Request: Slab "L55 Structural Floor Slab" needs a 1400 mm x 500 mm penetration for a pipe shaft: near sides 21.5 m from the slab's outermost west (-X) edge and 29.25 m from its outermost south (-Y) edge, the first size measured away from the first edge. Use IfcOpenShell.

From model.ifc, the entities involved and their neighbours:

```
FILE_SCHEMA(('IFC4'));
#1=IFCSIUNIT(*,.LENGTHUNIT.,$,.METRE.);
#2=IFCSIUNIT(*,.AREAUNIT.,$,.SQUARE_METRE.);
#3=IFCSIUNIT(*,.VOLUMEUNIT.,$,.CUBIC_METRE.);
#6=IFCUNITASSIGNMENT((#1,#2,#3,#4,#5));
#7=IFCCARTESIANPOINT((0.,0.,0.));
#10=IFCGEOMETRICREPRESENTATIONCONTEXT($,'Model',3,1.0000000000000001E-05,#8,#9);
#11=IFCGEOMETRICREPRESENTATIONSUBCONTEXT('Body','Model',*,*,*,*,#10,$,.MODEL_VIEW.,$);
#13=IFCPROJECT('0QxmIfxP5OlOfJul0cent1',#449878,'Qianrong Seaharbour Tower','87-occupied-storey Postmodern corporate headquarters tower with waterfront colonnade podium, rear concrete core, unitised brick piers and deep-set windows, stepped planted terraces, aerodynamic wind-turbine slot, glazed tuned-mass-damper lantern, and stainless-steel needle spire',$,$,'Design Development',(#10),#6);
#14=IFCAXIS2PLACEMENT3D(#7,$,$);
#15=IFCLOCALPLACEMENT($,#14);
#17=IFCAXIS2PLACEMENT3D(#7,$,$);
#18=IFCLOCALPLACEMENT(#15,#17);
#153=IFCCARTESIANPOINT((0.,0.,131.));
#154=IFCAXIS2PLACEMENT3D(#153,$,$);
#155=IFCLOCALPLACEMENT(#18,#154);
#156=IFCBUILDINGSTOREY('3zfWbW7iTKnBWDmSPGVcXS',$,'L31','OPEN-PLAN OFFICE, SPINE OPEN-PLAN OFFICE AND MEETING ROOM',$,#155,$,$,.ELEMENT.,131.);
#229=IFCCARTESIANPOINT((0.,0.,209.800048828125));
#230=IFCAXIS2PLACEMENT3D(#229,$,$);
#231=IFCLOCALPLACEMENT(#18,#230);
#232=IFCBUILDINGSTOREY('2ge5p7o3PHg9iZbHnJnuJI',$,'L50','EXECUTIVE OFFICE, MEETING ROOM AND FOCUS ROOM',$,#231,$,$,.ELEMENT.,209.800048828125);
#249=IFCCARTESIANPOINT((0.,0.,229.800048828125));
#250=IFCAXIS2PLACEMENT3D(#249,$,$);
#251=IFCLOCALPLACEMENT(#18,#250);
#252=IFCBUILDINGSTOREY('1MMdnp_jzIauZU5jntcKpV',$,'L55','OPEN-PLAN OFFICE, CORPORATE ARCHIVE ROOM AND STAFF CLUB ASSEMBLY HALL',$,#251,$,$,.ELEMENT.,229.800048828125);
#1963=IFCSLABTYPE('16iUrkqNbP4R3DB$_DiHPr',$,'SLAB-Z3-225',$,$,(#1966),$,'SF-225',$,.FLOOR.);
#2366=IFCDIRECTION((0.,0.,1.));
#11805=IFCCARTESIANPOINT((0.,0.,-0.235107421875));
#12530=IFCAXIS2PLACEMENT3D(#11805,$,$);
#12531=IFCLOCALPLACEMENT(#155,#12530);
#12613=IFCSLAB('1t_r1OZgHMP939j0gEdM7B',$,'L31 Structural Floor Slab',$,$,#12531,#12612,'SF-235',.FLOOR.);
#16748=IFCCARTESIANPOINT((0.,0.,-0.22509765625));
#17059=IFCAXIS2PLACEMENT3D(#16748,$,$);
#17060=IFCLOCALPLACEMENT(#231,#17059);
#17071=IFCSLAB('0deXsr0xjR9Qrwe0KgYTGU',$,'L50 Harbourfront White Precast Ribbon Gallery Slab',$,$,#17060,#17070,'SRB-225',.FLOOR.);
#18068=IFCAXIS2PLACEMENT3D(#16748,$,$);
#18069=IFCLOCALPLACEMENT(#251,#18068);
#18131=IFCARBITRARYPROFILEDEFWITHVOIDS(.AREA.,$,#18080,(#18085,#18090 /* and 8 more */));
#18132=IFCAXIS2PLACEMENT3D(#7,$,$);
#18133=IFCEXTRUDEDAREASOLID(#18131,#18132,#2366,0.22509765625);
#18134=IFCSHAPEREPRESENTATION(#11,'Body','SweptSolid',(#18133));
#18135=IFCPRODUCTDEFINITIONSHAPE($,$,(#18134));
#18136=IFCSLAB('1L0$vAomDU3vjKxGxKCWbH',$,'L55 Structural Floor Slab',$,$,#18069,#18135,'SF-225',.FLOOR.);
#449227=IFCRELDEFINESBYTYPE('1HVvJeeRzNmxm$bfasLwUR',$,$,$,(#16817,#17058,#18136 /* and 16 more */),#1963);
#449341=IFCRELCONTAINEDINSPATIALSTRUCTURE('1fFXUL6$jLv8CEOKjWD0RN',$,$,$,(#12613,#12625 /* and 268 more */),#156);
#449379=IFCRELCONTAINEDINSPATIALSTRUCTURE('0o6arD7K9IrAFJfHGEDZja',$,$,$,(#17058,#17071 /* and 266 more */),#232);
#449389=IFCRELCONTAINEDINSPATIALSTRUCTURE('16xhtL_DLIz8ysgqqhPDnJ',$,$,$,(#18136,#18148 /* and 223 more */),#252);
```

```python
import numpy as np
import ifcopenshell
import ifcopenshell.api.feature
import ifcopenshell.api.geometry
import ifcopenshell.api.root
import ifcopenshell.geom
import ifcopenshell.util.placement
import ifcopenshell.util.representation
import ifcopenshell.util.shape
import ifcopenshell.util.unit

model = ifcopenshell.open("model.ifc")
unit_scale = ifcopenshell.util.unit.calculate_unit_scale(model)
settings = ifcopenshell.geom.settings()


def volume(element):
    """Net volume in cubic metres, openings subtracted."""
    shape = ifcopenshell.geom.create_shape(settings, element)
    return ifcopenshell.util.shape.get_volume(shape.geometry)


slab = model.by_guid("1L0$vAomDU3vjKxGxKCWbH")
before = volume(slab)

# Extent in the slab's own axes, in metres. The edges named are its -X and -Y sides.
slab_shape = ifcopenshell.geom.create_shape(settings, slab)
vertices = ifcopenshell.util.shape.get_vertices(slab_shape.geometry)
x_min, y_min, bottom = vertices.min(axis=0)
top = vertices[:, 2].max()

opening = ifcopenshell.api.root.create_entity(model, ifc_class="IfcOpeningElement", name="Pipe shaft opening", predefined_type="OPENING")
context = ifcopenshell.util.representation.get_context(model, "Model", "Body", "MODEL_VIEW")
width, depth = 1.4, 0.5
outline = [(0.0, 0.0), (width, 0.0), (width, depth), (0.0, depth), (0.0, 0.0)]
# Overshoot both faces by 50 mm so the cut is clean.
shape = ifcopenshell.api.geometry.add_slab_representation(
    model, context=context, depth=top - bottom + 0.1, polyline=outline
)
ifcopenshell.api.geometry.assign_representation(model, product=opening, representation=shape)

matrix = ifcopenshell.util.placement.get_local_placement(slab.ObjectPlacement)
matrix[:, 3] = matrix @ np.append(np.array([x_min + 21.5, y_min + 29.25, bottom - 0.05]) / unit_scale, 1.0)
ifcopenshell.api.geometry.edit_object_placement(model, product=opening, matrix=matrix, is_si=False)
ifcopenshell.api.feature.add_feature(model, feature=opening, element=slab)

after = volume(slab)

print(f"slab volume {before:.3f} -> {after:.3f} m3")

model.write("model_edited.ifc")
```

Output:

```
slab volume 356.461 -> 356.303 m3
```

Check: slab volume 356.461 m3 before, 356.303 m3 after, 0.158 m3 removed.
